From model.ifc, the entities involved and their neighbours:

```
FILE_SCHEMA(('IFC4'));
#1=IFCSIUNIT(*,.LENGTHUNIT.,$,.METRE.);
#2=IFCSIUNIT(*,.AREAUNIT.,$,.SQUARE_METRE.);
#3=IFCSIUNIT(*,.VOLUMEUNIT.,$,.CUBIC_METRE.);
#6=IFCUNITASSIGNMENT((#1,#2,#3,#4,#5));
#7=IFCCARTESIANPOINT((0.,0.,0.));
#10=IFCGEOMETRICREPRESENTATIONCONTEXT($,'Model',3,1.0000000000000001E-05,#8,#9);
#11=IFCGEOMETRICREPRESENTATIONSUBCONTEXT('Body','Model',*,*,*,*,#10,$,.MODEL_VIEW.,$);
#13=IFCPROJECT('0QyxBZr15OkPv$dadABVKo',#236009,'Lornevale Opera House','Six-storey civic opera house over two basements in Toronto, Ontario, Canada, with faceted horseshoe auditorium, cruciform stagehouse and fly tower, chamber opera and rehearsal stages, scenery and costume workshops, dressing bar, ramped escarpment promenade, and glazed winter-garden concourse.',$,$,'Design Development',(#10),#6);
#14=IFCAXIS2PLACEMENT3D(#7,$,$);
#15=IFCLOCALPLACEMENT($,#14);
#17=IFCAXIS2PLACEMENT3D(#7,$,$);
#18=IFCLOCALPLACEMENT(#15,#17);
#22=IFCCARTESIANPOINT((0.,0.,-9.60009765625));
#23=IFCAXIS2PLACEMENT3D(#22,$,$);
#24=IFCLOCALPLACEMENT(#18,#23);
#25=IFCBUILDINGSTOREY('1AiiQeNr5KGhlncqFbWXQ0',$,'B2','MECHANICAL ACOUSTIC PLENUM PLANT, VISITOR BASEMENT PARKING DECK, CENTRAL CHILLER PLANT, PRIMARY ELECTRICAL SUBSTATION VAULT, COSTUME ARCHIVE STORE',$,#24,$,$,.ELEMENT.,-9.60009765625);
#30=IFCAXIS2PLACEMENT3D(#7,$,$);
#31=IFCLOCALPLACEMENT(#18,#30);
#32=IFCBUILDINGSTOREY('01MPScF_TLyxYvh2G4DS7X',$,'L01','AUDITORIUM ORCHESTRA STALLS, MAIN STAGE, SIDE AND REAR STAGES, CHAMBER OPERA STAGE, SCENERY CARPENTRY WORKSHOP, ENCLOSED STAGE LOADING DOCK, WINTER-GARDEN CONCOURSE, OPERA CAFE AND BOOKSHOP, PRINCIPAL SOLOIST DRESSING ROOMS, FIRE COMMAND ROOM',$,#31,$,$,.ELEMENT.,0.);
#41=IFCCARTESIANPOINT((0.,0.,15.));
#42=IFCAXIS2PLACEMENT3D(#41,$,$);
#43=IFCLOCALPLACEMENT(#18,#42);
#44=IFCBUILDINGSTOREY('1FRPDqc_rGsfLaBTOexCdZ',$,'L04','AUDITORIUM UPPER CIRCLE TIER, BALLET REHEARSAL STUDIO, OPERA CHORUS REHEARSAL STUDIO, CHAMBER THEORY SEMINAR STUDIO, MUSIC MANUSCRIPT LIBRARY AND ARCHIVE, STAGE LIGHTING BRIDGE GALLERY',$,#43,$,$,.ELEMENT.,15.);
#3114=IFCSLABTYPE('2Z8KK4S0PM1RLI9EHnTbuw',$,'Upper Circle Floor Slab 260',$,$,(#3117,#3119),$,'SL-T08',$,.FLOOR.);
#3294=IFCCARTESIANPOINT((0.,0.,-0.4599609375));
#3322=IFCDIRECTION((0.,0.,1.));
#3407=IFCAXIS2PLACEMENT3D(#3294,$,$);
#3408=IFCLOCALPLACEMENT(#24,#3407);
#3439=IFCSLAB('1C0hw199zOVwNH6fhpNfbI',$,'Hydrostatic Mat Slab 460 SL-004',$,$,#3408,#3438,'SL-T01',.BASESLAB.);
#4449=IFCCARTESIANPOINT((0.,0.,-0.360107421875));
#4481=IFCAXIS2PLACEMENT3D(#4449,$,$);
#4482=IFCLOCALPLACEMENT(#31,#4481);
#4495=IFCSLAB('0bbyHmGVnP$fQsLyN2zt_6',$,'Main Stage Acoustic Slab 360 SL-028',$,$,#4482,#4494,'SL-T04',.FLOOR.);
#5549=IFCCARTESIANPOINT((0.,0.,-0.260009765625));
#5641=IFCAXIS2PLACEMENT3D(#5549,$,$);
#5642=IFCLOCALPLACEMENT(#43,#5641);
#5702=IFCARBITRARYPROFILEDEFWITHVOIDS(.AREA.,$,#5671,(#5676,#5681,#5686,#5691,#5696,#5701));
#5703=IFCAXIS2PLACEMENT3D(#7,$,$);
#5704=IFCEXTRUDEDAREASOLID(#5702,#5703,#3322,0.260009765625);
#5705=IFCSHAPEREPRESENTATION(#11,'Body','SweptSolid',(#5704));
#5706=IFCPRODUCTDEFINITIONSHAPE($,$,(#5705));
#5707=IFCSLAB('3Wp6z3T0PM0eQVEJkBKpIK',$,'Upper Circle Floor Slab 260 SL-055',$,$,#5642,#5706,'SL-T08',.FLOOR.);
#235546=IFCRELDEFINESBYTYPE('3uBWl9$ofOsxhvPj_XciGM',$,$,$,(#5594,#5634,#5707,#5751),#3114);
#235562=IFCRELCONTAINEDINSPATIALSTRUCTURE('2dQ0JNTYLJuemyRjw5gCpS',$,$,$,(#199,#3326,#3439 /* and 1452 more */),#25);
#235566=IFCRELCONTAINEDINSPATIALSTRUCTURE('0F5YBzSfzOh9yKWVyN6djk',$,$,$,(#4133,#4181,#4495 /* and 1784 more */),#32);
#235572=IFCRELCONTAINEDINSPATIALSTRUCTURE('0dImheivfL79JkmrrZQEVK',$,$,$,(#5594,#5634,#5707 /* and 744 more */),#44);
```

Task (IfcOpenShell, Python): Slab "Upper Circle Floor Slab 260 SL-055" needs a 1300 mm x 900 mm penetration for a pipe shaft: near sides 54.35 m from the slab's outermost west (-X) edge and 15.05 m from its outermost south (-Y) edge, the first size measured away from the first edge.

```python
import numpy as np
import ifcopenshell
import ifcopenshell.api.feature
import ifcopenshell.api.geometry
import ifcopenshell.api.root
import ifcopenshell.geom
import ifcopenshell.util.placement
import ifcopenshell.util.representation
import ifcopenshell.util.shape
import ifcopenshell.util.unit

model = ifcopenshell.open("model.ifc")
unit_scale = ifcopenshell.util.unit.calculate_unit_scale(model)
settings = ifcopenshell.geom.settings()


def volume(element):
    """Net volume in cubic metres, openings subtracted."""
    shape = ifcopenshell.geom.create_shape(settings, element)
    return ifcopenshell.util.shape.get_volume(shape.geometry)


slab = model.by_guid("3Wp6z3T0PM0eQVEJkBKpIK")
before = volume(slab)

# Extent in the slab's own axes, in metres. The edges named are its -X and -Y sides.
slab_shape = ifcopenshell.geom.create_shape(settings, slab)
vertices = ifcopenshell.util.shape.get_vertices(slab_shape.geometry)
x_min, y_min, bottom = vertices.min(axis=0)
top = vertices[:, 2].max()

opening = ifcopenshell.api.root.create_entity(model, ifc_class="IfcOpeningElement", name="Pipe shaft opening", predefined_type="OPENING")
context = ifcopenshell.util.representation.get_context(model, "Model", "Body", "MODEL_VIEW")
width, depth = 1.3, 0.9
outline = [(0.0, 0.0), (width, 0.0), (width, depth), (0.0, depth), (0.0, 0.0)]
# Overshoot both faces by 50 mm so the cut is clean.
shape = ifcopenshell.api.geometry.add_slab_representation(
    model, context=context, depth=top - bottom + 0.1, polyline=outline
)
ifcopenshell.api.geometry.assign_representation(model, product=opening, representation=shape)

matrix = ifcopenshell.util.placement.get_local_placement(slab.ObjectPlacement)
matrix[:, 3] = matrix @ np.append(np.array([x_min + 54.35, y_min + 15.05, bottom - 0.05]) / unit_scale, 1.0)
ifcopenshell.api.geometry.edit_object_placement(model, product=opening, matrix=matrix, is_si=False)
ifcopenshell.api.feature.add_feature(model, feature=opening, element=slab)

after = volume(slab)

print(f"slab volume {before:.3f} -> {after:.3f} m3")

model.write("model_v2.ifc")
```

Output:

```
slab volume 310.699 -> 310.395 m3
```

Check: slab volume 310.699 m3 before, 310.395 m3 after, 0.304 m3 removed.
